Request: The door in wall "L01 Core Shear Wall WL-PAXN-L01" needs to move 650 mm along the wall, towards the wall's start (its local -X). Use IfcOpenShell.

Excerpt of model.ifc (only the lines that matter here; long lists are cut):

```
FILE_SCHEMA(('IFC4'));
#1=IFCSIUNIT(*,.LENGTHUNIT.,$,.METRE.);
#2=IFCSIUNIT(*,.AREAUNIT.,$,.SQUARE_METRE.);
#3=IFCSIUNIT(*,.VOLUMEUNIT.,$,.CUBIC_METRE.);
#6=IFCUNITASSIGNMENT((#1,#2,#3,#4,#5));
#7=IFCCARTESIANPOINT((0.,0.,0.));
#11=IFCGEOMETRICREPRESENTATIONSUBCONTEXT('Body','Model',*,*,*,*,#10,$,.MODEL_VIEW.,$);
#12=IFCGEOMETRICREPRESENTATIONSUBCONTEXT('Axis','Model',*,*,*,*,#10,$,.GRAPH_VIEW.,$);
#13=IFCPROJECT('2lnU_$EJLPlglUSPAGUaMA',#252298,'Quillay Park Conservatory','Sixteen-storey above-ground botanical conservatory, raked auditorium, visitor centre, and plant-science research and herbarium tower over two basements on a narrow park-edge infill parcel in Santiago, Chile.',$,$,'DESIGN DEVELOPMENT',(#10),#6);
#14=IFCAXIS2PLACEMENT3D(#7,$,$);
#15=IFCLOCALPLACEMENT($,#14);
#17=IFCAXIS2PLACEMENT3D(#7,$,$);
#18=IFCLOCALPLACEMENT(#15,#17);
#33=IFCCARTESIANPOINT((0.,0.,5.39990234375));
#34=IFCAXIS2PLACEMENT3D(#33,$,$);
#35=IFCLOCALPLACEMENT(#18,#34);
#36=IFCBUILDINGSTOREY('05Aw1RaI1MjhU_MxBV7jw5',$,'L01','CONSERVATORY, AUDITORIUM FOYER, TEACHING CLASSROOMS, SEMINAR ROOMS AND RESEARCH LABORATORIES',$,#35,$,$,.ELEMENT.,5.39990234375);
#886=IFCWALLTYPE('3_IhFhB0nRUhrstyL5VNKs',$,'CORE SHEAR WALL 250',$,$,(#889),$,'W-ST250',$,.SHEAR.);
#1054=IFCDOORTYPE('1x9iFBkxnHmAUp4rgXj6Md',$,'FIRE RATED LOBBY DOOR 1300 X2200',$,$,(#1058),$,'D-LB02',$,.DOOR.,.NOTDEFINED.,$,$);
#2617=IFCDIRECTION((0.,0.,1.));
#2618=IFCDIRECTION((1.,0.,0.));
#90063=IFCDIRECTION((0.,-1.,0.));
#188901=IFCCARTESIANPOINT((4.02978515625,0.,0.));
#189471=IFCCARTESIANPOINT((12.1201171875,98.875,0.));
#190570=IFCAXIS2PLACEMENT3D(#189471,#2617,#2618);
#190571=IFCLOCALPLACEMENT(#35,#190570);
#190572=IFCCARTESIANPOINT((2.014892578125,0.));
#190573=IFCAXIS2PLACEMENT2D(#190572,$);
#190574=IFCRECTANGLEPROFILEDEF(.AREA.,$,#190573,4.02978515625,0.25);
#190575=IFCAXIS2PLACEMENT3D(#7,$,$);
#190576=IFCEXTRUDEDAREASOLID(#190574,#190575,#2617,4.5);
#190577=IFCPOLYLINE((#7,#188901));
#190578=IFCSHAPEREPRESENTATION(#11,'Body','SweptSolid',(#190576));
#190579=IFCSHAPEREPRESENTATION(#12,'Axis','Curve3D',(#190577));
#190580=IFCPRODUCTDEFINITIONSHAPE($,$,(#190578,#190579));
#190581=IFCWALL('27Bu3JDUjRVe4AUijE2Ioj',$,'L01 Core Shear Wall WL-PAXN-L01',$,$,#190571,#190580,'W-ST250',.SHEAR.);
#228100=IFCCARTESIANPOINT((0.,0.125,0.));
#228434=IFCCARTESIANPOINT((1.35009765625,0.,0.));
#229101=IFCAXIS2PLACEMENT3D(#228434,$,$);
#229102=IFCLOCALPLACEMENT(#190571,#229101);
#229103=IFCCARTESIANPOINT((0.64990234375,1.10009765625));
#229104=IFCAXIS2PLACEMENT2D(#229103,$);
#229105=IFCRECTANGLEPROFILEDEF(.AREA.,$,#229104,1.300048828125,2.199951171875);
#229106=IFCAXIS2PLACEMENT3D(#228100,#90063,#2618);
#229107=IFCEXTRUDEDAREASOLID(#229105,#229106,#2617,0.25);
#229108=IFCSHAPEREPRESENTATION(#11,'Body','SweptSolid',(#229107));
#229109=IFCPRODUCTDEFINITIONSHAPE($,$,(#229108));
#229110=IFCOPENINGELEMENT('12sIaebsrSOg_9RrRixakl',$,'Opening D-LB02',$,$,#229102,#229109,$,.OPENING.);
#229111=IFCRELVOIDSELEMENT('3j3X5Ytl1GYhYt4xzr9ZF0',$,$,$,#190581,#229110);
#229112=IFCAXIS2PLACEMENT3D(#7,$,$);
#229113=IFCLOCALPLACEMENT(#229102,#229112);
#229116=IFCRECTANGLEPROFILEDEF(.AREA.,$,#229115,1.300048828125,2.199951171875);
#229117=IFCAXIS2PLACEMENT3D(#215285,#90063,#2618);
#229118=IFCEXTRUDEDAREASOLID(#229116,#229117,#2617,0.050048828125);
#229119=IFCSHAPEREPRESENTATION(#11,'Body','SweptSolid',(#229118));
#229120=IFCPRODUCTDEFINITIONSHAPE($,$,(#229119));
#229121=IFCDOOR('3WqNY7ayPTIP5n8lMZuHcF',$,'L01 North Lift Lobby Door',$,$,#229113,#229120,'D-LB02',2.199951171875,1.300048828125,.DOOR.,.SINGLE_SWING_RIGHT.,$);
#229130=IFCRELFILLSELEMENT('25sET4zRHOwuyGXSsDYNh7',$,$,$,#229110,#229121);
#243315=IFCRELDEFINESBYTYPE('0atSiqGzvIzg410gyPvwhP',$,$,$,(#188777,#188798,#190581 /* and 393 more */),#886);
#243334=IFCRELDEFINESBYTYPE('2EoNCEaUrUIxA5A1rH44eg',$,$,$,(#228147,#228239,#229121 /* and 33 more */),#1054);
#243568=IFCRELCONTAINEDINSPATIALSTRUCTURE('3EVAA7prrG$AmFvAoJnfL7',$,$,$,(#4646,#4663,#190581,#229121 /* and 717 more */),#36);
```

```python
import ifcopenshell
import ifcopenshell.api.geometry
import ifcopenshell.util.placement
import ifcopenshell.util.unit

model = ifcopenshell.open("model.ifc")
unit_scale = ifcopenshell.util.unit.calculate_unit_scale(model)

door = model.by_guid("3WqNY7ayPTIP5n8lMZuHcF")
opening = door.FillsVoids[0].RelatingOpeningElement
wall = opening.VoidsElements[0].RelatingBuildingElement

wall_matrix = ifcopenshell.util.placement.get_local_placement(wall.ObjectPlacement)
shift = wall_matrix[:3, 0] * -0.65 / unit_scale
before = ifcopenshell.util.placement.get_local_placement(door.ObjectPlacement)[:3, 3].copy()

# The door is placed relative to its opening, so it follows when the opening moves.
matrix = ifcopenshell.util.placement.get_local_placement(opening.ObjectPlacement)
matrix[:3, 3] += shift
ifcopenshell.api.geometry.edit_object_placement(
    model, product=opening, matrix=matrix, is_si=False, should_transform_children=True
)

after = ifcopenshell.util.placement.get_local_placement(door.ObjectPlacement)[:3, 3]
print("door moved by", (after - before).round(3) + 0.0)

model.write("model_updated.ifc")
```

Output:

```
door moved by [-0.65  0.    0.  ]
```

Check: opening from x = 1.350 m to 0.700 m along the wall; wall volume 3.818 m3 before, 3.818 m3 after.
